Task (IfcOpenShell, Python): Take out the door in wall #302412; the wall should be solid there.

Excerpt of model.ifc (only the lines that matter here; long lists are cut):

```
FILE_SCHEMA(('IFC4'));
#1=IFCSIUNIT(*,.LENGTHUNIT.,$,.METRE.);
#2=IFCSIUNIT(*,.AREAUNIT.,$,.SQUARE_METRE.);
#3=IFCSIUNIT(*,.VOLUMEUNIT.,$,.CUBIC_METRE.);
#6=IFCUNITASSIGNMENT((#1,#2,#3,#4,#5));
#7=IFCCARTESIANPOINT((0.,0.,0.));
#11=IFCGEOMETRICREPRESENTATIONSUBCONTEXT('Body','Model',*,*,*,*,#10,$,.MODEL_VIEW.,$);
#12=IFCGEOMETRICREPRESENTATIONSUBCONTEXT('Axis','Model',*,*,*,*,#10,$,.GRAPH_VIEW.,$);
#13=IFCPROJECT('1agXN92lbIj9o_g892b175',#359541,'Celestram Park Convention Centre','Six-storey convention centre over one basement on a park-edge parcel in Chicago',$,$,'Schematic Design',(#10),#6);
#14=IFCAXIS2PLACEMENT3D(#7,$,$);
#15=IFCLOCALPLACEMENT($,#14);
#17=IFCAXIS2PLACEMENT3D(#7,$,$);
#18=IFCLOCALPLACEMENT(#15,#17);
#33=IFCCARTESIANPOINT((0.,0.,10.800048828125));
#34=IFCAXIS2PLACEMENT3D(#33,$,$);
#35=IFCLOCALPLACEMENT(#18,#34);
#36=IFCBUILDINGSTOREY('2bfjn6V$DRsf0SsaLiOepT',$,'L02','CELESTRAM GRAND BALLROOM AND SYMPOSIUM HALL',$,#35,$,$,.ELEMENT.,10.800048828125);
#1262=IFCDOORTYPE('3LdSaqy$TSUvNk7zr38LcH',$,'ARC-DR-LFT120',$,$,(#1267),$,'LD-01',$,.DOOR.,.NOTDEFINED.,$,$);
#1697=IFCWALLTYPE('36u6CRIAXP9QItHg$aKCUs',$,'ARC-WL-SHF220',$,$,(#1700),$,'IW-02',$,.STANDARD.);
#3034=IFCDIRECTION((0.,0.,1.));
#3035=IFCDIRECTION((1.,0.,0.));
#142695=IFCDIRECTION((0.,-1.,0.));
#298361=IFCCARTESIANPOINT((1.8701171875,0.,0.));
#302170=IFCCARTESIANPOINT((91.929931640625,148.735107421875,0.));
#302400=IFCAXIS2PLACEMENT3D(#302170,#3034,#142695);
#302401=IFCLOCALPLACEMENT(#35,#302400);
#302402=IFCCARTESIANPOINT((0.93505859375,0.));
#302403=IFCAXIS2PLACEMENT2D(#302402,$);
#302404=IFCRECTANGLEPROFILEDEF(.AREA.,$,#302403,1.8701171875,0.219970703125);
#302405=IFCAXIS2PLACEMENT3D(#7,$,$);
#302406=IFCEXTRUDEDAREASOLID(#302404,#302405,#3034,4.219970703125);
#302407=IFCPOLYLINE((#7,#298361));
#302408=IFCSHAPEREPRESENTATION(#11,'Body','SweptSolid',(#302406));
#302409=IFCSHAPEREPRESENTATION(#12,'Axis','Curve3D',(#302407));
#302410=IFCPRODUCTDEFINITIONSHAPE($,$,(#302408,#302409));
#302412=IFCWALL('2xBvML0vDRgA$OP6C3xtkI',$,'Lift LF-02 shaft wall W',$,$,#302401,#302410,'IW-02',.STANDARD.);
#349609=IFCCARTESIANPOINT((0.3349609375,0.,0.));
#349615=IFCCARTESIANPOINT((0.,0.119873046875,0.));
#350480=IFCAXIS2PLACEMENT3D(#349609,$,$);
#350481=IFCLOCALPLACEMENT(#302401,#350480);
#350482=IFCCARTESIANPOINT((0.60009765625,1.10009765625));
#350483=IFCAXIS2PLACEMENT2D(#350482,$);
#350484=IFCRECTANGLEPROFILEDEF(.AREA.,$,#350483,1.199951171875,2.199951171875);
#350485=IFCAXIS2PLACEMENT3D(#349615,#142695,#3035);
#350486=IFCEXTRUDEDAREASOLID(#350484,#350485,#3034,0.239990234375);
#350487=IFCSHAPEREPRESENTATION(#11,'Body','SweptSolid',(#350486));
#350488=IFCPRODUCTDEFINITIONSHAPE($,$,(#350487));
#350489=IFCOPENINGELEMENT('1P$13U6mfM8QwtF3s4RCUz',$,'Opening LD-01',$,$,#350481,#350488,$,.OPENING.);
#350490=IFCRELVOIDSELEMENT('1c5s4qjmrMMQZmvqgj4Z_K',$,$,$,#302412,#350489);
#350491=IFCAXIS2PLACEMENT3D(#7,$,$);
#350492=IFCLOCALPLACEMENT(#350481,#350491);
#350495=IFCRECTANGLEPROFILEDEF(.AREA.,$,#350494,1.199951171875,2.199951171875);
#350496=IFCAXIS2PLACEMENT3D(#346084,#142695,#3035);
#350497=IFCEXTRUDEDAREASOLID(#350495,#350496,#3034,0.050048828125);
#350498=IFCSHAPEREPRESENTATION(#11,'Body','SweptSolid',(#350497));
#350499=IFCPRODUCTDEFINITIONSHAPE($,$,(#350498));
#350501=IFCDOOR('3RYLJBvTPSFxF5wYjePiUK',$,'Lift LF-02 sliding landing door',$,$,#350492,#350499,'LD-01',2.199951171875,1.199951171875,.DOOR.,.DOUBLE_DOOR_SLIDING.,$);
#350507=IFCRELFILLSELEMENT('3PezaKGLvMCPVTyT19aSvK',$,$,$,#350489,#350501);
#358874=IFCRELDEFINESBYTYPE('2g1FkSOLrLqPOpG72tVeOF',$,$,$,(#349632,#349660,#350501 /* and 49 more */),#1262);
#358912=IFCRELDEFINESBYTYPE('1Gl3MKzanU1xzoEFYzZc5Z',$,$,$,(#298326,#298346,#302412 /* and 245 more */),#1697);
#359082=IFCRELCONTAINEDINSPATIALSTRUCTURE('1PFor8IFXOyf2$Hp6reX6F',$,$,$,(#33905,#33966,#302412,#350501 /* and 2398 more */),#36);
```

```python
import ifcopenshell
import ifcopenshell.api.feature
import ifcopenshell.api.root
import ifcopenshell.geom
import ifcopenshell.util.shape

model = ifcopenshell.open("model.ifc")
settings = ifcopenshell.geom.settings()


def volume(element):
    """Net volume in cubic metres, openings subtracted."""
    shape = ifcopenshell.geom.create_shape(settings, element)
    return ifcopenshell.util.shape.get_volume(shape.geometry)


door = model.by_guid("3RYLJBvTPSFxF5wYjePiUK")
opening = door.FillsVoids[0].RelatingOpeningElement
wall = opening.VoidsElements[0].RelatingBuildingElement
before = volume(wall)

ifcopenshell.api.root.remove_product(model, product=door)
ifcopenshell.api.feature.remove_feature(model, feature=opening)

after = volume(wall)

print(f"wall volume {before:.3f} -> {after:.3f} m3")

model.write("model-out.ifc")
```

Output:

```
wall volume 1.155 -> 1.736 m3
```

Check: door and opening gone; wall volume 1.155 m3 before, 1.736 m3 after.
